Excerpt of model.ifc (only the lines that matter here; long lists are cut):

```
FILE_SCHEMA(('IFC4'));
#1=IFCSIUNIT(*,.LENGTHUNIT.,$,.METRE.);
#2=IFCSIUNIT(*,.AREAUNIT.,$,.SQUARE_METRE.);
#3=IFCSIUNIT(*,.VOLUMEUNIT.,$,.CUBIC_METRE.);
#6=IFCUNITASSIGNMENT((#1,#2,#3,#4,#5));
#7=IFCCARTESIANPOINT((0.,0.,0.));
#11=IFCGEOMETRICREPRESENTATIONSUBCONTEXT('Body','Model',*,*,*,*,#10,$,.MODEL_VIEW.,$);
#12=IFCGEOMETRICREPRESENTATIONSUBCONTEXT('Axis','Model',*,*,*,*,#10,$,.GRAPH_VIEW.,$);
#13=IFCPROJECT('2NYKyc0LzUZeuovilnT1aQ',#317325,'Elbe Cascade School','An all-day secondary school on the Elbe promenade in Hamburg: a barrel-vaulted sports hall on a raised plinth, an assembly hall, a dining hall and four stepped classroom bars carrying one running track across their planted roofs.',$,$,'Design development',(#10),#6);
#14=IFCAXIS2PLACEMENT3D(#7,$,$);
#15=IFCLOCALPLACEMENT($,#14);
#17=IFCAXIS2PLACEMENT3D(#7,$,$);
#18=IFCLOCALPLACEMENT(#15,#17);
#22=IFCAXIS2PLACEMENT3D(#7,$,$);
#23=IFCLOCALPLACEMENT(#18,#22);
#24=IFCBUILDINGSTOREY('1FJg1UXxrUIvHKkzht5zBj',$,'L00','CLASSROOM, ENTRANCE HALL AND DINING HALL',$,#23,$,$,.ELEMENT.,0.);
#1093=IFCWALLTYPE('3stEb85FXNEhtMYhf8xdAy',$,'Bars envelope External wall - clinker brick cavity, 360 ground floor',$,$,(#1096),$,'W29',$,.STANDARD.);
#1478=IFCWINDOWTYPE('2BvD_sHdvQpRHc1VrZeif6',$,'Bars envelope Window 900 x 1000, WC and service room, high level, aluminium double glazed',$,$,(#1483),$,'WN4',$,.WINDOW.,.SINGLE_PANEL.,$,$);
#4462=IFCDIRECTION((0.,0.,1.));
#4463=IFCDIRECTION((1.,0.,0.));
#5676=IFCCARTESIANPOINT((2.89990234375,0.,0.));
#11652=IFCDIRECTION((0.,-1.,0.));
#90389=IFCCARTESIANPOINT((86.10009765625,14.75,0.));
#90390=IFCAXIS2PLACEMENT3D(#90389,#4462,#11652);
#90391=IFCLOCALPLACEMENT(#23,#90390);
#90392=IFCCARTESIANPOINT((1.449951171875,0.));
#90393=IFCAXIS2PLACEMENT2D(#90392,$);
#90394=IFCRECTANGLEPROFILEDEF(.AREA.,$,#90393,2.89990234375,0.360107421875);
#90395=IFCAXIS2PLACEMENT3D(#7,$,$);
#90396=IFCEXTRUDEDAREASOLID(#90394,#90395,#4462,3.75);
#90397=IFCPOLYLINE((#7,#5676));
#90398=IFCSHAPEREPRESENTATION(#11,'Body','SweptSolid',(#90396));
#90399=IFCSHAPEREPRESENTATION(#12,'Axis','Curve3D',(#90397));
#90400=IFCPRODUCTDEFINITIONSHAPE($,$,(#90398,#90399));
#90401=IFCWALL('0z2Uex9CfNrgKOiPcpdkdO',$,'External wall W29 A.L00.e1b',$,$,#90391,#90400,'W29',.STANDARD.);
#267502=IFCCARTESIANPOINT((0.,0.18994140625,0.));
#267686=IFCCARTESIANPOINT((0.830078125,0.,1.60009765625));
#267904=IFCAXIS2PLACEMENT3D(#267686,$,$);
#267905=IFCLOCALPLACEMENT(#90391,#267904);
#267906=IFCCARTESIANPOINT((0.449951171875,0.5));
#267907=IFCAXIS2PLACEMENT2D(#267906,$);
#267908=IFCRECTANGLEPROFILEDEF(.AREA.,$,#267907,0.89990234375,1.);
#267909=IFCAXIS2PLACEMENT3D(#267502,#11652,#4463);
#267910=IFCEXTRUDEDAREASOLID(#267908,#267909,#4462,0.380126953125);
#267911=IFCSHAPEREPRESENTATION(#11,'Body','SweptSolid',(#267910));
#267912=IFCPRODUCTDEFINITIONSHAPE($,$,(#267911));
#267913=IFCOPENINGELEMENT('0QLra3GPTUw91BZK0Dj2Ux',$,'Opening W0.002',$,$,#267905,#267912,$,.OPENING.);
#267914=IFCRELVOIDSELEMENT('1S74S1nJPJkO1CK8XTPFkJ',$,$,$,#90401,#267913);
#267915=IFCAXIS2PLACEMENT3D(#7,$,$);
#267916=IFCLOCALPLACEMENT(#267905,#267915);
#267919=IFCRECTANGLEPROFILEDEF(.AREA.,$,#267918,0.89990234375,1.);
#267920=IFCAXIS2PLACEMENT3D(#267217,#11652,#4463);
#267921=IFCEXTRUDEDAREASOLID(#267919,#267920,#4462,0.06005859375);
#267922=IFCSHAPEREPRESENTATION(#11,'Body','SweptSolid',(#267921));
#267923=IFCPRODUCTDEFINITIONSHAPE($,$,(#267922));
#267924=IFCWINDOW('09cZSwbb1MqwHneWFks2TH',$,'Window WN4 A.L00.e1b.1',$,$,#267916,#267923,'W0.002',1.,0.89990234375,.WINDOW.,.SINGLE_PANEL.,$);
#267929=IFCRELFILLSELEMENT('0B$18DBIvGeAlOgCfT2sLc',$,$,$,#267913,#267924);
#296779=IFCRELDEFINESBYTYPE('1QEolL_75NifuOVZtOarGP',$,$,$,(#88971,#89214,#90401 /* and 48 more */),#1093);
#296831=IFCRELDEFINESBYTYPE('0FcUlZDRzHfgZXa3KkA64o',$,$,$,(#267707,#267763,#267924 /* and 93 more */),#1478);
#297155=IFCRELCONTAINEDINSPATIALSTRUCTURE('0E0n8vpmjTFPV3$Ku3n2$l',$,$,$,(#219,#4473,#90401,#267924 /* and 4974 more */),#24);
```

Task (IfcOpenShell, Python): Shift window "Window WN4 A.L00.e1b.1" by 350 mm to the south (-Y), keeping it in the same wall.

```python
import ifcopenshell
import ifcopenshell.api.geometry
import ifcopenshell.util.placement
import ifcopenshell.util.unit

model = ifcopenshell.open("model.ifc")
unit_scale = ifcopenshell.util.unit.calculate_unit_scale(model)

window = model.by_id(267924)
opening = window.FillsVoids[0].RelatingOpeningElement
wall = opening.VoidsElements[0].RelatingBuildingElement

wall_matrix = ifcopenshell.util.placement.get_local_placement(wall.ObjectPlacement)
shift = wall_matrix[:3, 0] * 0.35 / unit_scale
before = ifcopenshell.util.placement.get_local_placement(window.ObjectPlacement)[:3, 3].copy()

# The window is placed relative to its opening, so it follows when the opening moves.
matrix = ifcopenshell.util.placement.get_local_placement(opening.ObjectPlacement)
matrix[:3, 3] += shift
ifcopenshell.api.geometry.edit_object_placement(
    model, product=opening, matrix=matrix, is_si=False, should_transform_children=True
)

after = ifcopenshell.util.placement.get_local_placement(window.ObjectPlacement)[:3, 3]
print("window moved by", (after - before).round(3) + 0.0)

model.write("model-out.ifc")
```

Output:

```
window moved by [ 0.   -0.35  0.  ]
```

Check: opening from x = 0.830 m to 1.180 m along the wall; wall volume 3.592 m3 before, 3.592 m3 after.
